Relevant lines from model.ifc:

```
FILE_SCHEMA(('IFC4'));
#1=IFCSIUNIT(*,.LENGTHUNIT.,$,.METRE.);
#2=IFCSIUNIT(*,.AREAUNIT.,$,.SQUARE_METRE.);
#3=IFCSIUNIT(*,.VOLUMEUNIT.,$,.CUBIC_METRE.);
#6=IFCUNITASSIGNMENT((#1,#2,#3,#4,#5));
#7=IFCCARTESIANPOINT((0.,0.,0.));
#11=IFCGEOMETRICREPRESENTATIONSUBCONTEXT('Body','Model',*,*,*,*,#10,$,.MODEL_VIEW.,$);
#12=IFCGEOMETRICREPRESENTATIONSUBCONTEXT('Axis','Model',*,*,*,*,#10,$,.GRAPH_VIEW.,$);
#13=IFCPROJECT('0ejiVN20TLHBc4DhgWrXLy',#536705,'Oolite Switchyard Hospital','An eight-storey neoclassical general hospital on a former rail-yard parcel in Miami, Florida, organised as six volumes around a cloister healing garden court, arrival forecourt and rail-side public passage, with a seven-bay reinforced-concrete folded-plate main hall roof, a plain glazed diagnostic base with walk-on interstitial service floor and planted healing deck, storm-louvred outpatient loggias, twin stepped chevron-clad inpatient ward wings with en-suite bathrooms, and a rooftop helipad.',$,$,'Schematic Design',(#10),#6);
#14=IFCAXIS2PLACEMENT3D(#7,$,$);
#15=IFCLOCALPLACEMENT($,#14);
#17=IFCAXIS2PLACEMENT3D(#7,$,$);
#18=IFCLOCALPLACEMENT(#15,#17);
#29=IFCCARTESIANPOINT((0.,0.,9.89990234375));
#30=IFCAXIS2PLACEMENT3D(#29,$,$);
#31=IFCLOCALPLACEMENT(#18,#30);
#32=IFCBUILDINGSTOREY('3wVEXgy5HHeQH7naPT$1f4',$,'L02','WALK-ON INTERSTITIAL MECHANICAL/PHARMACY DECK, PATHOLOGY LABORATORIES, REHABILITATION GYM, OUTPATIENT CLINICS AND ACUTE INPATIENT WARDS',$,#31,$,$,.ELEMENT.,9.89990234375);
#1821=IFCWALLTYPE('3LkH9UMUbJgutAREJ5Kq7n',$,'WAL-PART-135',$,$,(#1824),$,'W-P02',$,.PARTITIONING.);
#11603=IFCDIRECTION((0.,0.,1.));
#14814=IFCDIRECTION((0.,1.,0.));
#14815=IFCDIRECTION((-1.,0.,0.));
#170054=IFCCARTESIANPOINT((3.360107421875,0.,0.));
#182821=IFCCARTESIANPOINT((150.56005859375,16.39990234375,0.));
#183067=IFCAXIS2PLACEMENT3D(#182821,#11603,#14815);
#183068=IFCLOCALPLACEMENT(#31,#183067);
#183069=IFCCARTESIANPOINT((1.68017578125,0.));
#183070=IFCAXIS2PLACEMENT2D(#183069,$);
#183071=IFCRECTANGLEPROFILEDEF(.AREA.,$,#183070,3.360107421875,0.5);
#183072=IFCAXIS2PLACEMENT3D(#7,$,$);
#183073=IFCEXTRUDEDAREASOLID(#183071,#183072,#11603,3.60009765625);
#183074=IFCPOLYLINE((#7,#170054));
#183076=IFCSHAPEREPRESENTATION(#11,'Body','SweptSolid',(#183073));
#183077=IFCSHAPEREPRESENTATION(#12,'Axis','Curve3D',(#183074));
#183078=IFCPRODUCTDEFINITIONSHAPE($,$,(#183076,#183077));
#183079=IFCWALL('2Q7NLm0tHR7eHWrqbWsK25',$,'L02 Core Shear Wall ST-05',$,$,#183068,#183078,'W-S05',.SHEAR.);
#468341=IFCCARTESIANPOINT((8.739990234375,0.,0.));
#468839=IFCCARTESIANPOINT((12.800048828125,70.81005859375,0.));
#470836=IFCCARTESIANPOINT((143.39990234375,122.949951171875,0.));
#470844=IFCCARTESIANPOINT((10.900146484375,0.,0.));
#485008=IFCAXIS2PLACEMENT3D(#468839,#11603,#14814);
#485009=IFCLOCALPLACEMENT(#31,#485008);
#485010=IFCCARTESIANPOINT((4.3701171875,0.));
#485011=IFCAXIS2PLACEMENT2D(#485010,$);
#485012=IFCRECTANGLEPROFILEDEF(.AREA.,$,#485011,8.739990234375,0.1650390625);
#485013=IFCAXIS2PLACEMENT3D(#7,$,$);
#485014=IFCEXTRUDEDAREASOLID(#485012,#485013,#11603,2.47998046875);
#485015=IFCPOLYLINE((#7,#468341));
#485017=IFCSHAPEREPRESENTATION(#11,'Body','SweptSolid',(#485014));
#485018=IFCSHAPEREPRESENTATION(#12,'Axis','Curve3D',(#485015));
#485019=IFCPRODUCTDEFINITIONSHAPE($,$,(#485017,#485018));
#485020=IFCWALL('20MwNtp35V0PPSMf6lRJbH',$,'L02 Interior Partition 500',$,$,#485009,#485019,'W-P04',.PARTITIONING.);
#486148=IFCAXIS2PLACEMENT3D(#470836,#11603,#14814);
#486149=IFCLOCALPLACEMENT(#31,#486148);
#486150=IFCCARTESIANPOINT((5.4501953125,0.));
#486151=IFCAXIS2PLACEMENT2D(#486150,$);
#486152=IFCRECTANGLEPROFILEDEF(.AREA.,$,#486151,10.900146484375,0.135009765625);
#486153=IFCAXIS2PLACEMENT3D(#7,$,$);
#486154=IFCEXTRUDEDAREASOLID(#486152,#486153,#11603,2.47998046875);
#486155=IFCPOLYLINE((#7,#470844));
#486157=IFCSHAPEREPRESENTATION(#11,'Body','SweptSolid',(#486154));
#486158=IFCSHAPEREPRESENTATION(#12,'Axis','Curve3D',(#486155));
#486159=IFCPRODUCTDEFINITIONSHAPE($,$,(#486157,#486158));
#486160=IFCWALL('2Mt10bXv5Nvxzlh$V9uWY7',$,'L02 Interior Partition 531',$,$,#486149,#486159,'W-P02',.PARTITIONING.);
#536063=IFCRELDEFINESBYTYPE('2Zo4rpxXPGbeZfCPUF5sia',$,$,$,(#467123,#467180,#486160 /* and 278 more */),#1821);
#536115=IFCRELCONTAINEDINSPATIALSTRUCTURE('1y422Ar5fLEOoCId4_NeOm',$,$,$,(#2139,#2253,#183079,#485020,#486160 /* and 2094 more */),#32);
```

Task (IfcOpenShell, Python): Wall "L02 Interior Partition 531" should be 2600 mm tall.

```python
import ifcopenshell
import ifcopenshell.geom
import ifcopenshell.util.representation
import ifcopenshell.util.shape
import ifcopenshell.util.unit

model = ifcopenshell.open("model.ifc")
unit_scale = ifcopenshell.util.unit.calculate_unit_scale(model)
settings = ifcopenshell.geom.settings()


def volume(element):
    """Net volume in cubic metres, openings subtracted."""
    shape = ifcopenshell.geom.create_shape(settings, element)
    return ifcopenshell.util.shape.get_volume(shape.geometry)


wall = model.by_guid("2Mt10bXv5Nvxzlh$V9uWY7")
before = volume(wall)

body = ifcopenshell.util.representation.get_representation(wall, "Model", "Body")
solid = body.Items[0]
old_height = solid.Depth
solid.Depth = 2.6 / unit_scale
after = volume(wall)

print(f"height {old_height:g} -> {solid.Depth:g}, volume {before:.3f} -> {after:.3f} m3")

model.write("model_rev.ifc")
```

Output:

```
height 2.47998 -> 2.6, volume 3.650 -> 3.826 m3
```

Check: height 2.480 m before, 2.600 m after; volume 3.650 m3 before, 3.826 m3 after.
